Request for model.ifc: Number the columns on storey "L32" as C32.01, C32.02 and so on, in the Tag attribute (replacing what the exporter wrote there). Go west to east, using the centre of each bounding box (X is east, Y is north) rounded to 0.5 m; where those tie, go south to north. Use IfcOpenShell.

First a look at what the model holds.

```python
import ifcopenshell
import ifcopenshell.util.element
import ifcopenshell.util.placement

model = ifcopenshell.open("model.ifc")
print(model.schema)
storey = next(s for s in model.by_type("IfcBuildingStorey") if s.Name == "L32")
columns = [e for e in ifcopenshell.util.element.get_decomposition(storey) if e.is_a("IfcColumn")]
for e in sorted(columns, key=lambda e: e.id()):
    origin = ifcopenshell.util.placement.get_local_placement(e.ObjectPlacement)[:3, 3]
    print(e.id(), e.Tag, e.Name, origin.round(2) + 0.0, sep=" | ")
```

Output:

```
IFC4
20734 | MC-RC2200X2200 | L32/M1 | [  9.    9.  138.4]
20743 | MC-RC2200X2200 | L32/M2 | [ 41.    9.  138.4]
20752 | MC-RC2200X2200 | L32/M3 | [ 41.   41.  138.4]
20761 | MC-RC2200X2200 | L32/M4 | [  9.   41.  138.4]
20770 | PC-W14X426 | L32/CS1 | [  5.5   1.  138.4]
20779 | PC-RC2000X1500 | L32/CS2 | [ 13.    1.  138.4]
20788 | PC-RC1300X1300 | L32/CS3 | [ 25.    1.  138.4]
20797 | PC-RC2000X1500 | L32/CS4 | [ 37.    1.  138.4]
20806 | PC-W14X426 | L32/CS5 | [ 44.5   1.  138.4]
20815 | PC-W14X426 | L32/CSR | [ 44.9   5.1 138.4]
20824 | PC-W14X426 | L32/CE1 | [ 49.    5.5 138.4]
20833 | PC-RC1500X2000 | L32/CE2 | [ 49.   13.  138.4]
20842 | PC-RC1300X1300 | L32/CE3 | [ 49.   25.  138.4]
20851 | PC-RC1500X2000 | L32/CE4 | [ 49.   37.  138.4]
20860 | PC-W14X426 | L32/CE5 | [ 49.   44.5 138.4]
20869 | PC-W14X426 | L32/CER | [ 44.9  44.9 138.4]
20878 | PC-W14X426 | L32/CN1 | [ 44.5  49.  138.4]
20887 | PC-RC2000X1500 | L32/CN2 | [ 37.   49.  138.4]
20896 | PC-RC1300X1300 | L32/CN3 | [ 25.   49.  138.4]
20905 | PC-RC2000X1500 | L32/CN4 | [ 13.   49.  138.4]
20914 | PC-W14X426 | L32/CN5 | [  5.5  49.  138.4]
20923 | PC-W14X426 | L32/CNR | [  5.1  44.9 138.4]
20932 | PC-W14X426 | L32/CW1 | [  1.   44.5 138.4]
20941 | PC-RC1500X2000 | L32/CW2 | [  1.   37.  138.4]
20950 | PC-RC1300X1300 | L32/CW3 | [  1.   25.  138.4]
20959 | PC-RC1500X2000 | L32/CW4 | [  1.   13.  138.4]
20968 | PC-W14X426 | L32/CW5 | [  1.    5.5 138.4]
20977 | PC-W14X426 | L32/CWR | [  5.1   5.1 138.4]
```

```python
import ifcopenshell
import ifcopenshell.geom
import ifcopenshell.util.element
import ifcopenshell.util.shape

model = ifcopenshell.open("model.ifc")
settings = ifcopenshell.geom.settings()
settings.set("use-world-coords", True)


def centre(element):
    shape = ifcopenshell.geom.create_shape(settings, element)
    return ifcopenshell.util.shape.get_bbox_centroid(shape.geometry)


storey = next(s for s in model.by_type("IfcBuildingStorey") if s.Name == "L32")
columns = [e for e in ifcopenshell.util.element.get_decomposition(storey) if e.is_a("IfcColumn")]

# Insertion points can sit at a corner or the storey origin, so sort by the geometry (in metres).
centres = {e: centre(e) for e in columns}
columns.sort(key=lambda e: (round(centres[e][0] / 0.5), centres[e][1]))

for i, e in enumerate(columns, start=1):
    number = f"C32.{i:02d}"
    e.Tag = number
    print(e.id(), number)

model.write("model-out.ifc")
```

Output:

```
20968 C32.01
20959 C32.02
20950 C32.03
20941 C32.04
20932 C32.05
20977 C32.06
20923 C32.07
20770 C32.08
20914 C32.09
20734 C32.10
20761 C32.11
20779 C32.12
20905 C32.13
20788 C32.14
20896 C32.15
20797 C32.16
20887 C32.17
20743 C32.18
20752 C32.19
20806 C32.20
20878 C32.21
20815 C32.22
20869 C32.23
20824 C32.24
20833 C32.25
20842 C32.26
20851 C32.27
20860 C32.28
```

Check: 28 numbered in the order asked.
